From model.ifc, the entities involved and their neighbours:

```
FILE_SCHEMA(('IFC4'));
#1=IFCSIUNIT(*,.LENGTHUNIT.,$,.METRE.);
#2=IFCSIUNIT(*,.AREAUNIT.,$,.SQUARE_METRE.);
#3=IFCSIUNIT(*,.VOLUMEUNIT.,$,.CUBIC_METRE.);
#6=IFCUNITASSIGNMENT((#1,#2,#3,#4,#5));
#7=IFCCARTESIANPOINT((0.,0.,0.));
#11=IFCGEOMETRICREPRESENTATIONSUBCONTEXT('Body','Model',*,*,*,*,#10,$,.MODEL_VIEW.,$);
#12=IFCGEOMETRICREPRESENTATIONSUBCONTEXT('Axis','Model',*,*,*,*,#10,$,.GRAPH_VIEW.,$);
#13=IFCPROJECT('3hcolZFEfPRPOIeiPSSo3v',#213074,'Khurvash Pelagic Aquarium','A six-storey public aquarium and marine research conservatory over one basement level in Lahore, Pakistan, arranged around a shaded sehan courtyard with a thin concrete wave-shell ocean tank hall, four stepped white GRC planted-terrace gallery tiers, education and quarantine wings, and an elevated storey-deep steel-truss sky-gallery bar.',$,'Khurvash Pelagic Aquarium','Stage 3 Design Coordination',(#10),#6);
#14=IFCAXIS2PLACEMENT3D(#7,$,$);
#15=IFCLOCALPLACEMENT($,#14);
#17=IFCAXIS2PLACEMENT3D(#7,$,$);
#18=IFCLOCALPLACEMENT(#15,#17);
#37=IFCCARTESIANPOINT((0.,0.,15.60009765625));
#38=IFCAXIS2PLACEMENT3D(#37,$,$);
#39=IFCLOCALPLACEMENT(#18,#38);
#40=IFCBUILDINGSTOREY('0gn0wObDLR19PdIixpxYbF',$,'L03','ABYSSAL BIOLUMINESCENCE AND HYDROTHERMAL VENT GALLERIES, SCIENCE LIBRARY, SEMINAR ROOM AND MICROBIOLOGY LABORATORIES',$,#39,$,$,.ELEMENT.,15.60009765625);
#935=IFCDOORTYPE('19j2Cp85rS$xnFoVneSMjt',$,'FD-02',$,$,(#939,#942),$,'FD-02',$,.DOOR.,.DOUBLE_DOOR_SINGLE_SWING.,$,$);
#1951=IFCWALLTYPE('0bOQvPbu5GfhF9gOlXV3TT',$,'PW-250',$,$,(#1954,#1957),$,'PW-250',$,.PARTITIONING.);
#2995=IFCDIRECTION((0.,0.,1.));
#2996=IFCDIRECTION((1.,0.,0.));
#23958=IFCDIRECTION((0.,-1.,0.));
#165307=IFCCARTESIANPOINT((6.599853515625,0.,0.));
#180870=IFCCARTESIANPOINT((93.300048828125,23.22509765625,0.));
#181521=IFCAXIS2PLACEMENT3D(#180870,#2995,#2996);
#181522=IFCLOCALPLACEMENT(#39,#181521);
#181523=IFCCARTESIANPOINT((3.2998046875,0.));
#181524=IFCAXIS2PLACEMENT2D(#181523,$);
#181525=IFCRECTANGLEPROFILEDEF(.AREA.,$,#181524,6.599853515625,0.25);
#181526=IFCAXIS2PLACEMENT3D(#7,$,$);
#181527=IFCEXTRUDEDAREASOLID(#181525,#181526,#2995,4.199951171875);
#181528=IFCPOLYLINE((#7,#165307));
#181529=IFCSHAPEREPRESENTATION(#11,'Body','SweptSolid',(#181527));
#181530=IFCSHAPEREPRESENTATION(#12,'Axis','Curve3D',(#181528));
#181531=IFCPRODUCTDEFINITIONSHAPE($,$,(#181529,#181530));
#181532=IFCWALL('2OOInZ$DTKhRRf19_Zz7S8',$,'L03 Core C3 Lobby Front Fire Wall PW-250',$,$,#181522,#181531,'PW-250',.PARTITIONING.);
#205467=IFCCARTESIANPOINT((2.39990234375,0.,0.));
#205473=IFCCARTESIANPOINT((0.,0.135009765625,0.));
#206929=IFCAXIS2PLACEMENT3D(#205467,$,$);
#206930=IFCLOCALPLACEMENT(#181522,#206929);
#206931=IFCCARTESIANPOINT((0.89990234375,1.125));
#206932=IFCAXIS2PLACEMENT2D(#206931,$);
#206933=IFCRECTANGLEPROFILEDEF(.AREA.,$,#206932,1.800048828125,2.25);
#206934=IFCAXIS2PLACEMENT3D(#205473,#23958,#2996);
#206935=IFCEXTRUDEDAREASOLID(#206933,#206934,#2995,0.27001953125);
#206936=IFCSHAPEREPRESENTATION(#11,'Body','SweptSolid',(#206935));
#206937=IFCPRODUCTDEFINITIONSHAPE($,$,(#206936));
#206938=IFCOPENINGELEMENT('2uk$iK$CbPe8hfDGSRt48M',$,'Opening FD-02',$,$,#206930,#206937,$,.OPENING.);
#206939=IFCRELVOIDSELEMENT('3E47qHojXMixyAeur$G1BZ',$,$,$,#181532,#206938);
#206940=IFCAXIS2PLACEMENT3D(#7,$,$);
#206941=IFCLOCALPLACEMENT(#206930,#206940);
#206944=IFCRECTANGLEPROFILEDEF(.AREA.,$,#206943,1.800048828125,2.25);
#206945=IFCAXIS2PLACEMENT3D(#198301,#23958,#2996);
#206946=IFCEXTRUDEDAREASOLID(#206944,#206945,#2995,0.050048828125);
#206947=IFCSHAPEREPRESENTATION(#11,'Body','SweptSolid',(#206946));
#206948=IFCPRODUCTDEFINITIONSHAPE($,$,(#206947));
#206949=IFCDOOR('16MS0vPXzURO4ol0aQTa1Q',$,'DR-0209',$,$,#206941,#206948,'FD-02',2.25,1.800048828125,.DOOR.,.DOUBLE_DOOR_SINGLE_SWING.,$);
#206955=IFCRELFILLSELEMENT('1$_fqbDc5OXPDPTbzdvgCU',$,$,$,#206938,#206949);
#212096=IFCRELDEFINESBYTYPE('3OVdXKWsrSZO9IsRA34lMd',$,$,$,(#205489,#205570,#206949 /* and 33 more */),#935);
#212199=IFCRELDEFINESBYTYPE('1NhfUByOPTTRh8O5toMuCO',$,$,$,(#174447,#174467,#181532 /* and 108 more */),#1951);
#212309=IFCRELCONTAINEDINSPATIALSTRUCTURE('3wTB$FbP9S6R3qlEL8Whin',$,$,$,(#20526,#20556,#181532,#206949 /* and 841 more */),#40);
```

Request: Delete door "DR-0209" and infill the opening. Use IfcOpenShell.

```python
import ifcopenshell
import ifcopenshell.api.feature
import ifcopenshell.api.root
import ifcopenshell.geom
import ifcopenshell.util.shape

model = ifcopenshell.open("model.ifc")
settings = ifcopenshell.geom.settings()


def volume(element):
    """Net volume in cubic metres, openings subtracted."""
    shape = ifcopenshell.geom.create_shape(settings, element)
    return ifcopenshell.util.shape.get_volume(shape.geometry)


door = model.by_guid("16MS0vPXzURO4ol0aQTa1Q")
opening = door.FillsVoids[0].RelatingOpeningElement
wall = opening.VoidsElements[0].RelatingBuildingElement
before = volume(wall)

ifcopenshell.api.root.remove_product(model, product=door)
ifcopenshell.api.feature.remove_feature(model, feature=opening)

after = volume(wall)

print(f"wall volume {before:.3f} -> {after:.3f} m3")

model.write("model_v2.ifc")
```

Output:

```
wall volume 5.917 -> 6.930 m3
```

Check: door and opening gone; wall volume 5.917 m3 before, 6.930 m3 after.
